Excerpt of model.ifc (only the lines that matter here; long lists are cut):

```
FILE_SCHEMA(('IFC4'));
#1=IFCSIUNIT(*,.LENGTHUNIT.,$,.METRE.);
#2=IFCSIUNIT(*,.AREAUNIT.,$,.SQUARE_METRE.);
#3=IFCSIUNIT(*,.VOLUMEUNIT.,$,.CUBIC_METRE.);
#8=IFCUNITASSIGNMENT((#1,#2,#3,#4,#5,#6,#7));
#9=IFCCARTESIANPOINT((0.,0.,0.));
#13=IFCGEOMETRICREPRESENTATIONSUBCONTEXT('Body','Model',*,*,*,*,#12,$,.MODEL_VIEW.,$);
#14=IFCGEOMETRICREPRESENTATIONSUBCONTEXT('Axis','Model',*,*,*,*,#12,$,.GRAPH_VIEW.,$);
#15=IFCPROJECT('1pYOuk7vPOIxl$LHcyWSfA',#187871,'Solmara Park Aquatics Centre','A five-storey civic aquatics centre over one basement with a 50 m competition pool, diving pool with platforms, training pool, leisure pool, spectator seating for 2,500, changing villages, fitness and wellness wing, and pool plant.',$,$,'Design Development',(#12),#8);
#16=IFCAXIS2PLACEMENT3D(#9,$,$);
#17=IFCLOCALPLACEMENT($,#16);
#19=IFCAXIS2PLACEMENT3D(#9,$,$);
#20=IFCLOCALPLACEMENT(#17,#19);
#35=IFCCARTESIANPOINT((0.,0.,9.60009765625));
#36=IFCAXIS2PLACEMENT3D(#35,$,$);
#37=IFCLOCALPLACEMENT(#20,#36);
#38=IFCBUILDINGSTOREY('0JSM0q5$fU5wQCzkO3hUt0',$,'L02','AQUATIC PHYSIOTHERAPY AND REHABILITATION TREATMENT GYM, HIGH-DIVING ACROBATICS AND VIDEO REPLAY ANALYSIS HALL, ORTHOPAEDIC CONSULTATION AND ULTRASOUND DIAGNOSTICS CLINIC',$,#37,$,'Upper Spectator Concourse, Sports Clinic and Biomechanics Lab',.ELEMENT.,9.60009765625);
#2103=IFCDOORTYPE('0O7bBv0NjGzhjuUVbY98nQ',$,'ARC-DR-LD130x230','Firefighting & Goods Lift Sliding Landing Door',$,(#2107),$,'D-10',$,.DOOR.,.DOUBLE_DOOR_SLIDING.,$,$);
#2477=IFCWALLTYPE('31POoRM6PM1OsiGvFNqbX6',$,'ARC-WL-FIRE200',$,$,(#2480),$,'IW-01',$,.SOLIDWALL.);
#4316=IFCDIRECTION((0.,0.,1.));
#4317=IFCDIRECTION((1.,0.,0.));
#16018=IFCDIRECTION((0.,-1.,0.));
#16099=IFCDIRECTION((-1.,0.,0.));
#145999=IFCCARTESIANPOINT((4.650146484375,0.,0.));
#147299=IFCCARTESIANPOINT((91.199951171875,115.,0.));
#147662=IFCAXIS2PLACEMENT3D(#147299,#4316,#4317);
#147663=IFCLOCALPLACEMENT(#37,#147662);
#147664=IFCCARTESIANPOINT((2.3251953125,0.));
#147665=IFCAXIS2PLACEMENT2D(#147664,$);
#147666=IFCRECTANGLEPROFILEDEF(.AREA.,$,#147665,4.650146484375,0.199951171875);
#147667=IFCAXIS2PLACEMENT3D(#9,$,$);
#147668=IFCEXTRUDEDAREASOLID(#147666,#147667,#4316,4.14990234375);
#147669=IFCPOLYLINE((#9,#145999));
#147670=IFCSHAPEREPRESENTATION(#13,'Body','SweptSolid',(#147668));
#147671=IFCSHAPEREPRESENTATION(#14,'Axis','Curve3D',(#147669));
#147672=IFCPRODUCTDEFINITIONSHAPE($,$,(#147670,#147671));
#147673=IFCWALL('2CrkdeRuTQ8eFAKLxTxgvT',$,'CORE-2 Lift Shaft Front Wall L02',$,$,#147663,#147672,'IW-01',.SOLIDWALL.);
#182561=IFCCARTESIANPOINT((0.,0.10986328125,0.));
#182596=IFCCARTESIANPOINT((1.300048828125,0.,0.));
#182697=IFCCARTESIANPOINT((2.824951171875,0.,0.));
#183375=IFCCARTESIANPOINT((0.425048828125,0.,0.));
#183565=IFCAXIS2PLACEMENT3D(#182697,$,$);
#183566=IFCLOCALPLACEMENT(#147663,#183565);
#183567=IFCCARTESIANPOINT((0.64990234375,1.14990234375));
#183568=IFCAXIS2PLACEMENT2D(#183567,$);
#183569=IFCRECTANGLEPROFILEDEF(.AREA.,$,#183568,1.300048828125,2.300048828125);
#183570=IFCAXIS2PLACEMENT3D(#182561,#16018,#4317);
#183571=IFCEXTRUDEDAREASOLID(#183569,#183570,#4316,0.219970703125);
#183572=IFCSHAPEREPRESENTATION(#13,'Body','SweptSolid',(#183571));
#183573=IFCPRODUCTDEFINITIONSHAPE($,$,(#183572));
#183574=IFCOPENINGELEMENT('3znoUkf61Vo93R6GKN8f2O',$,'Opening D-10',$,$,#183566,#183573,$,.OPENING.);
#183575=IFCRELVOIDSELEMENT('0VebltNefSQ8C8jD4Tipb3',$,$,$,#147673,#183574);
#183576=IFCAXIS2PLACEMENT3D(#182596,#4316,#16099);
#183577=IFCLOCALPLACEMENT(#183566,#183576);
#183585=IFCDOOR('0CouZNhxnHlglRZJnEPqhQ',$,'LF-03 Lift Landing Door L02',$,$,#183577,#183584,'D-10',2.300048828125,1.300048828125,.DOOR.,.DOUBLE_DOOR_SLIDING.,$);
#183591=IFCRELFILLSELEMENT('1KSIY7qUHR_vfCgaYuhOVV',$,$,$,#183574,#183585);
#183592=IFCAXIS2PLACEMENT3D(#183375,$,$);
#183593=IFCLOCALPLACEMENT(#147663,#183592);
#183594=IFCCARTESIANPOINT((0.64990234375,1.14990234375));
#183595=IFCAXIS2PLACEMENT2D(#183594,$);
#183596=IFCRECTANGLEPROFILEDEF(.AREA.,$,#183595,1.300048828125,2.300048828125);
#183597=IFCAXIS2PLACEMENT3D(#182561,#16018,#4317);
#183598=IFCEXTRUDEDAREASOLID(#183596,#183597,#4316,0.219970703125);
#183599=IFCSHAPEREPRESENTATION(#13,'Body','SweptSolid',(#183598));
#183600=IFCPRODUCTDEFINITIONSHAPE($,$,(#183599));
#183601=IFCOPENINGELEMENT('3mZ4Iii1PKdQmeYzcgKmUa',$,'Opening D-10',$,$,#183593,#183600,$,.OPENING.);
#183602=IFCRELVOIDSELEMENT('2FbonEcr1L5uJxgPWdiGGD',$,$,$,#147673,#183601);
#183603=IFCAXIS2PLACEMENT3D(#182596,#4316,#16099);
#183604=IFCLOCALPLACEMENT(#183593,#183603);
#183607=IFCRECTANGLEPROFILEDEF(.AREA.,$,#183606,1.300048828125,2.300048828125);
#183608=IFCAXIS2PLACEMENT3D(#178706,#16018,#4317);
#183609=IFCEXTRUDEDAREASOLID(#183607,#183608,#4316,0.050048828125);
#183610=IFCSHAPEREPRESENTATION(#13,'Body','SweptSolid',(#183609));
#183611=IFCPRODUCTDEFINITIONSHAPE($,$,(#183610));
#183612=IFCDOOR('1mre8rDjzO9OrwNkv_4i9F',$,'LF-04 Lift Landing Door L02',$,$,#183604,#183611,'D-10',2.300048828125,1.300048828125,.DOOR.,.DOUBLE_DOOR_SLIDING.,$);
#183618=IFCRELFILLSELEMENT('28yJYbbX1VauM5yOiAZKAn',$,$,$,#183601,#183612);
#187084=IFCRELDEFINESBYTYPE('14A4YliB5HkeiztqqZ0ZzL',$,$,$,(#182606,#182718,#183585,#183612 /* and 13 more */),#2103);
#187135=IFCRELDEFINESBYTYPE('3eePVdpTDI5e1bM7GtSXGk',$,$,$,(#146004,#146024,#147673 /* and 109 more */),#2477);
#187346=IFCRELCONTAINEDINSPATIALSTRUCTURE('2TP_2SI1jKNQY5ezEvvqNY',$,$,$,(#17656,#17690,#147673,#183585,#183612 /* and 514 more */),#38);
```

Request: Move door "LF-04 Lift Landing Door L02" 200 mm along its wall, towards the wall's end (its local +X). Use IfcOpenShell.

```python
import ifcopenshell
import ifcopenshell.api.geometry
import ifcopenshell.util.placement

model = ifcopenshell.open("model.ifc")

door = model.by_guid("1mre8rDjzO9OrwNkv_4i9F")
opening = door.FillsVoids[0].RelatingOpeningElement
wall = opening.VoidsElements[0].RelatingBuildingElement

wall_matrix = ifcopenshell.util.placement.get_local_placement(wall.ObjectPlacement)
shift = wall_matrix[:3, 0] * 0.2
before = ifcopenshell.util.placement.get_local_placement(door.ObjectPlacement)[:3, 3].copy()

# The door is placed relative to its opening, so it follows when the opening moves.
matrix = ifcopenshell.util.placement.get_local_placement(opening.ObjectPlacement)
matrix[:3, 3] += shift
ifcopenshell.api.geometry.edit_object_placement(
    model, product=opening, matrix=matrix, is_si=False, should_transform_children=True
)

after = ifcopenshell.util.placement.get_local_placement(door.ObjectPlacement)[:3, 3]
print("door moved by", (after - before).round(3) + 0.0)

model.write("model_updated.ifc")
```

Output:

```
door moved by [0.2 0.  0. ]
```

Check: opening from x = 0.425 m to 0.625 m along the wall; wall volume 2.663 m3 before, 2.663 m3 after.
